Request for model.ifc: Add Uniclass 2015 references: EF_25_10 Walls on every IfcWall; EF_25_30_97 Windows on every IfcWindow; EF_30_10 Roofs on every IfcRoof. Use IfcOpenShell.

First a look at what the model holds.

```python
import ifcopenshell

model = ifcopenshell.open("model.ifc")
print(model.schema)
print("classifications:", [c.Name for c in model.by_type("IfcClassification")])
for ifc_class in ("IfcDoor", "IfcRoof", "IfcStair", "IfcWall", "IfcWindow"):
    print(ifc_class, len(model.by_type(ifc_class)))
```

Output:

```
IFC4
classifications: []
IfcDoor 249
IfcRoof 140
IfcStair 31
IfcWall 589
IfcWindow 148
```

```python
import ifcopenshell
import ifcopenshell.api.classification

model = ifcopenshell.open("model.ifc")

system = ifcopenshell.api.classification.add_classification(model, classification="Uniclass 2015")

codes = {
    "IfcWall": ("EF_25_10", "Walls"),
    "IfcWindow": ("EF_25_30_97", "Windows"),
    "IfcRoof": ("EF_30_10", "Roofs"),
}
for ifc_class, (code, name) in codes.items():
    products = model.by_type(ifc_class)
    ifcopenshell.api.classification.add_reference(
        model, products=products, classification=system, identification=code, name=name
    )
    print(code, len(products))

model.write("model_edited.ifc")
```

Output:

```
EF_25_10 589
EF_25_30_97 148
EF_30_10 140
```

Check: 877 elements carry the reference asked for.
